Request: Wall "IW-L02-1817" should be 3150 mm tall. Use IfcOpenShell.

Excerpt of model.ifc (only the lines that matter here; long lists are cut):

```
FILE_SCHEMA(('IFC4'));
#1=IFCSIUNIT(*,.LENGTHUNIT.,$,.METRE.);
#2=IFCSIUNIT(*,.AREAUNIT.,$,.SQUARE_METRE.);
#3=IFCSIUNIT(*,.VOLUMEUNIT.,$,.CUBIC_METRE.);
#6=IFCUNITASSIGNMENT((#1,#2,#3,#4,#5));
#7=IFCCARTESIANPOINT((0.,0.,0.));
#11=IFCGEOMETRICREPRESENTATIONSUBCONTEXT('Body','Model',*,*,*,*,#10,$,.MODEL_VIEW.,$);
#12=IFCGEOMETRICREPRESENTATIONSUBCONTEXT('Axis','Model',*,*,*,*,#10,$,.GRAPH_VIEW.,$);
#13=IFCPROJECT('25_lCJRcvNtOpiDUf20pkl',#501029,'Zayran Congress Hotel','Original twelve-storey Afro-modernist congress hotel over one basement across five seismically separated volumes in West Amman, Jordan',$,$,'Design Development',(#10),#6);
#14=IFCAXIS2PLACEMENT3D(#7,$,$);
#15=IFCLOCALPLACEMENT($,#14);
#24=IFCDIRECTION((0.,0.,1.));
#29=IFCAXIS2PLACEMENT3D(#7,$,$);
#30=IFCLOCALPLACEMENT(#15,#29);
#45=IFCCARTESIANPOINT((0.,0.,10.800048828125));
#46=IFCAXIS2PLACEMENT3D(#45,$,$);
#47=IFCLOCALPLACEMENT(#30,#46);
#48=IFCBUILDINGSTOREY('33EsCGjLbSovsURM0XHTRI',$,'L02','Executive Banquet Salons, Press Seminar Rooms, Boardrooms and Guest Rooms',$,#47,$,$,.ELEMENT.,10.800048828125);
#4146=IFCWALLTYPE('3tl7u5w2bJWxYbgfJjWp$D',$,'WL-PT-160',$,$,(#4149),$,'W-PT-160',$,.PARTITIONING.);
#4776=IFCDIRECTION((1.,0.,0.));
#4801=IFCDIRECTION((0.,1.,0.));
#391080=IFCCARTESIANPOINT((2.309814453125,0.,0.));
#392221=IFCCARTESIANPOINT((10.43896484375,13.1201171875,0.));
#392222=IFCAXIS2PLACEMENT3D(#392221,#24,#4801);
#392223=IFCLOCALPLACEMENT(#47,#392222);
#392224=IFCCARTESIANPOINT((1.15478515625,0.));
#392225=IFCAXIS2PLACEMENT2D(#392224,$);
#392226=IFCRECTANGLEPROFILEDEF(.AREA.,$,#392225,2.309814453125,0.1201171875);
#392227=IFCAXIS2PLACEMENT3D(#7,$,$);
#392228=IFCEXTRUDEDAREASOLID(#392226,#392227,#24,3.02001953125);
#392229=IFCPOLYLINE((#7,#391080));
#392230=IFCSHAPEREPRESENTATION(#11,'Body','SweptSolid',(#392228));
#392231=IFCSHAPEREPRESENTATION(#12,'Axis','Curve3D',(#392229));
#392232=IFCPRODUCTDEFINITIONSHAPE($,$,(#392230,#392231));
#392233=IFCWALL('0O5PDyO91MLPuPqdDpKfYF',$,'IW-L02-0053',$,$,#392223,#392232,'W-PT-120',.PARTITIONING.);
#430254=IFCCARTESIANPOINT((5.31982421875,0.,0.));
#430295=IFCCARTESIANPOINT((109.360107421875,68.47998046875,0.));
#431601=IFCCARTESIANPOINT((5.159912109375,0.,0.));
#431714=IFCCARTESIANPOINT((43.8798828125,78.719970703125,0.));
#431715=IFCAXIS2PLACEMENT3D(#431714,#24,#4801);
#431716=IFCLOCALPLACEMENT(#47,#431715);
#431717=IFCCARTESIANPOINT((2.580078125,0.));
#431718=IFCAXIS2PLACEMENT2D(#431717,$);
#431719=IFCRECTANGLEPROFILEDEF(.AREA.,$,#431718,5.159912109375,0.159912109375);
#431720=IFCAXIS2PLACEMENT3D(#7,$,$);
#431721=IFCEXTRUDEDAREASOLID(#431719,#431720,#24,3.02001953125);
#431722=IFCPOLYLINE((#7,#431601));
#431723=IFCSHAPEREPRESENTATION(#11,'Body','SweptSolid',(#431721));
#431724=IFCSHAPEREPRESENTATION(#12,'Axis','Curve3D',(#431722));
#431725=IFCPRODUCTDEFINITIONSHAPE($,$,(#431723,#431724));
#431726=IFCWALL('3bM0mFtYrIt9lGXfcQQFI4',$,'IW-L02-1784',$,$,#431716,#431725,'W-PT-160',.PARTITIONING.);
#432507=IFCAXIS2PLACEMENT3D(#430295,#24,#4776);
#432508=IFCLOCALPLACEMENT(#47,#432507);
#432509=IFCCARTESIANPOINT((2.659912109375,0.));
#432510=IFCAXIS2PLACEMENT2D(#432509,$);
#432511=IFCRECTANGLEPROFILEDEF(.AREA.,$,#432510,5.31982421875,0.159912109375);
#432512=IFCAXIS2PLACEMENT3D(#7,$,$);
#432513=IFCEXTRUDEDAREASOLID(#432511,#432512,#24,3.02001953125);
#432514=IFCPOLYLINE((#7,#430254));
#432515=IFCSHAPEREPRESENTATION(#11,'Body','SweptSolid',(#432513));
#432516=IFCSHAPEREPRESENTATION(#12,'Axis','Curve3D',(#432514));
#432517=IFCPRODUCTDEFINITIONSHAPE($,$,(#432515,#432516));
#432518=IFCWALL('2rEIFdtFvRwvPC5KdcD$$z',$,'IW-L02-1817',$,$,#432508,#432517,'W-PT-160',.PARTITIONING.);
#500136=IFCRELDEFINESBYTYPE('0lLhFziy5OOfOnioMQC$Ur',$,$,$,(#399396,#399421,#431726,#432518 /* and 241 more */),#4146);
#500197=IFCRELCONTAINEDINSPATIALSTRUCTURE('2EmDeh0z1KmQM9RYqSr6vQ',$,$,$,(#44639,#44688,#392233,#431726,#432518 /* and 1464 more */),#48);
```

```python
import ifcopenshell
import ifcopenshell.geom
import ifcopenshell.util.representation
import ifcopenshell.util.shape

model = ifcopenshell.open("model.ifc")
settings = ifcopenshell.geom.settings()


def volume(element):
    """Net volume in cubic metres, openings subtracted."""
    shape = ifcopenshell.geom.create_shape(settings, element)
    return ifcopenshell.util.shape.get_volume(shape.geometry)


wall = model.by_id(432518)
before = volume(wall)

body = ifcopenshell.util.representation.get_representation(wall, "Model", "Body")
solid = body.Items[0]
old_height = solid.Depth
solid.Depth = 3.15
after = volume(wall)

print(f"height {old_height:g} -> {solid.Depth:g}, volume {before:.3f} -> {after:.3f} m3")

model.write("model_edited.ifc")
```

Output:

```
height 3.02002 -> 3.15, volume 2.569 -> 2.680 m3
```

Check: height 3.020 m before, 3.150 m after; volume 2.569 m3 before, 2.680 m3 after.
